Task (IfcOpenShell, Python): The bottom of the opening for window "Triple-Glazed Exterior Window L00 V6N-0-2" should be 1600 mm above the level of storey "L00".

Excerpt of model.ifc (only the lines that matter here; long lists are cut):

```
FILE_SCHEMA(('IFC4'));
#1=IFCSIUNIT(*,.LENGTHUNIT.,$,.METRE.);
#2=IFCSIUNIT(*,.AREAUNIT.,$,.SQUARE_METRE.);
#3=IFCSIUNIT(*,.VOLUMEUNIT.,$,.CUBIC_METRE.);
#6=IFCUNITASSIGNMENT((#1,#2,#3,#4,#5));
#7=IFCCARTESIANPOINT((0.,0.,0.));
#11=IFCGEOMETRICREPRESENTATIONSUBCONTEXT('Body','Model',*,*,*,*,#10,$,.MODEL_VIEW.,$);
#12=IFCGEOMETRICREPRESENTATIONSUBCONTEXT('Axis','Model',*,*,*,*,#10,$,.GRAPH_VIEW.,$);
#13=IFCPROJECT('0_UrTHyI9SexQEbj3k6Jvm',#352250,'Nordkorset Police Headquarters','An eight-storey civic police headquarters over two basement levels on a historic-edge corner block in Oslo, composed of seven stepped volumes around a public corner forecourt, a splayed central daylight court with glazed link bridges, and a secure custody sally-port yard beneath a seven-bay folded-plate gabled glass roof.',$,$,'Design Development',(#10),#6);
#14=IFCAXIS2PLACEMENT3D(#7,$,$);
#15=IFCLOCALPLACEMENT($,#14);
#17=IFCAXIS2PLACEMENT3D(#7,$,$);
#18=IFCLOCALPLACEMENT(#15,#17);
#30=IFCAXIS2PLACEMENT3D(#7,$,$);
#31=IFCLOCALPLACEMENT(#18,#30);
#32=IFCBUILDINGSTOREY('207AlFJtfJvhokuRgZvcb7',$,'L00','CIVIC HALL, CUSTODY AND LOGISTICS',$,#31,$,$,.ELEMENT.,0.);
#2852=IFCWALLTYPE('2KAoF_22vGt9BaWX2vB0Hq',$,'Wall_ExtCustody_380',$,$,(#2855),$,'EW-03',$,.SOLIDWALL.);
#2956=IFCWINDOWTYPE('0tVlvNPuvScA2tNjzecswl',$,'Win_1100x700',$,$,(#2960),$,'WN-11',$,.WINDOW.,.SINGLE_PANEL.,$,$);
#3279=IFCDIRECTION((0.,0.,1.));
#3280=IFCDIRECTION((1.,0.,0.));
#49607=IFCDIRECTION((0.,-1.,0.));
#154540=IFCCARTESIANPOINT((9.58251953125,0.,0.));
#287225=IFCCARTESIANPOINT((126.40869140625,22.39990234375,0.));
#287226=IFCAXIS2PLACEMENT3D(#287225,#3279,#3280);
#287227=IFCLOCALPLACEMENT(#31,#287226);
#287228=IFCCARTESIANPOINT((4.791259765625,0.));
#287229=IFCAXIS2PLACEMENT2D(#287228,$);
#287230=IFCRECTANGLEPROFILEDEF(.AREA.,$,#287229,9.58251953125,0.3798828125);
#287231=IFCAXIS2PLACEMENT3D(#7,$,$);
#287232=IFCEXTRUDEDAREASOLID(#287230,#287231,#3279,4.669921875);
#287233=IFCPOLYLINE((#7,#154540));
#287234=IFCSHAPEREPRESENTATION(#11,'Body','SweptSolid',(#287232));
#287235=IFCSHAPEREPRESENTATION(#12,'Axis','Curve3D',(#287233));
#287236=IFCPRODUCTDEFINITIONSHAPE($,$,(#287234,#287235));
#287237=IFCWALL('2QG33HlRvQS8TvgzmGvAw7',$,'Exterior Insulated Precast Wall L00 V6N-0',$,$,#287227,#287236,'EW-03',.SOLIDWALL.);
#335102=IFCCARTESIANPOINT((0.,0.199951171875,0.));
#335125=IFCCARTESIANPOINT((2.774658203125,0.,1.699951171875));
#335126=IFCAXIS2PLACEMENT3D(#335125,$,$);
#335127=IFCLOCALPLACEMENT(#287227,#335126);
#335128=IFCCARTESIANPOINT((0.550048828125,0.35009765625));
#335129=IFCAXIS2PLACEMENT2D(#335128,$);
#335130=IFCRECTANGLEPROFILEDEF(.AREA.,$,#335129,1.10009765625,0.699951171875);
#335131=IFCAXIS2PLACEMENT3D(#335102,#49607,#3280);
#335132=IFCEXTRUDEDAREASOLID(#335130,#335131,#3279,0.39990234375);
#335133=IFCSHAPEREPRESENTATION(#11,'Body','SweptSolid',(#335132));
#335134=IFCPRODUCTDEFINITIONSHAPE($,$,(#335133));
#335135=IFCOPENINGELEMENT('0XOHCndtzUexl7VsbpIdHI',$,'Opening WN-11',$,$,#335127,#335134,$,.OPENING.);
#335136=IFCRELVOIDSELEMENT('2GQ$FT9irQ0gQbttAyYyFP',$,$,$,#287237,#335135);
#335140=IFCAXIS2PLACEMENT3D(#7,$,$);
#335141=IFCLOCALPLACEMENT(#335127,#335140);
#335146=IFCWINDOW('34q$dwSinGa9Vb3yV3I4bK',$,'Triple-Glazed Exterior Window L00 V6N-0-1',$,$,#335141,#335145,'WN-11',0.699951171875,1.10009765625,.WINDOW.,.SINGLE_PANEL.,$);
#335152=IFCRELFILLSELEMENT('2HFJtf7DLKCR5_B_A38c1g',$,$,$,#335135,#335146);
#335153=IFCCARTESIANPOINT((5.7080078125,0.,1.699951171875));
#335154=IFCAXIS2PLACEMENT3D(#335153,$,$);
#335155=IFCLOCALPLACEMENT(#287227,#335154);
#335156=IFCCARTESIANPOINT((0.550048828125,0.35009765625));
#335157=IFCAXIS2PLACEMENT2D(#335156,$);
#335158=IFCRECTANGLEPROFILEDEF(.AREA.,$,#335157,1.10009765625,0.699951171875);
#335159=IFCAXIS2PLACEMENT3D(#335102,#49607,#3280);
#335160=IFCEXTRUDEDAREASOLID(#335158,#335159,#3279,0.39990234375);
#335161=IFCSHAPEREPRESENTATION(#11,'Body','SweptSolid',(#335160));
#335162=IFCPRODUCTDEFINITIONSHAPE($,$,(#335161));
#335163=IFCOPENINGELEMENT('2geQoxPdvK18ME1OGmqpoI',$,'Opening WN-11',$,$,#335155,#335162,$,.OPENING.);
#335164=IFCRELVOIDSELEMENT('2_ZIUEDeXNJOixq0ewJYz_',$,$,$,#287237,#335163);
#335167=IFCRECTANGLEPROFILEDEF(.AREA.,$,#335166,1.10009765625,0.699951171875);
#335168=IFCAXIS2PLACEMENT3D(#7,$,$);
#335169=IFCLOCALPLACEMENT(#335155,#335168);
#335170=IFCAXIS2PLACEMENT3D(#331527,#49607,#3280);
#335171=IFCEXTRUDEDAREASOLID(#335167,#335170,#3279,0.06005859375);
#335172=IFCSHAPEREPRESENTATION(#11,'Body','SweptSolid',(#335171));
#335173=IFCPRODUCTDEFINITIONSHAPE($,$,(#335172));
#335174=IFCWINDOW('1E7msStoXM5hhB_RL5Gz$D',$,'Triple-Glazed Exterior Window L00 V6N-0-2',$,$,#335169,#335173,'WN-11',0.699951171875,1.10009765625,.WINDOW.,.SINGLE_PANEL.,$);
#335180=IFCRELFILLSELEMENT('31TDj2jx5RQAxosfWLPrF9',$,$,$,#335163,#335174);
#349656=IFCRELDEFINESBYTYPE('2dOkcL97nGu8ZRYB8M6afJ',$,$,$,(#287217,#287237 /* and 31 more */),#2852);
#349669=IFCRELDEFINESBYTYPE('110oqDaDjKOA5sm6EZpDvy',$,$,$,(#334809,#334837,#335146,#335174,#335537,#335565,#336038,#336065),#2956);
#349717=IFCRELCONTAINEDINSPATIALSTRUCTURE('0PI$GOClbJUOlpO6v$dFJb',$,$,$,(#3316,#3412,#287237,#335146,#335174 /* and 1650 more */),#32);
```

```python
import numpy as np
import ifcopenshell
import ifcopenshell.api.geometry
import ifcopenshell.geom
import ifcopenshell.util.element
import ifcopenshell.util.placement
import ifcopenshell.util.shape
import ifcopenshell.util.unit

model = ifcopenshell.open("model.ifc")
unit_scale = ifcopenshell.util.unit.calculate_unit_scale(model)

window = model.by_guid("1E7msStoXM5hhB_RL5Gz$D")
opening = window.FillsVoids[0].RelatingOpeningElement
storey = ifcopenshell.util.element.get_container(window, ifc_class="IfcBuildingStorey")
level = ifcopenshell.util.placement.get_local_placement(storey.ObjectPlacement)[2, 3]

# The opening's origin need not be at the sill, so measure its lowest point.
shape = ifcopenshell.geom.create_shape(ifcopenshell.geom.settings(), opening)
bottom = ifcopenshell.util.shape.get_shape_bottom_elevation(shape, shape.geometry) / unit_scale
dz = level + 1.6 / unit_scale - bottom

shift = np.array([0.0, 0.0, dz])
# The window is placed relative to its opening, so it follows when the opening moves.
matrix = ifcopenshell.util.placement.get_local_placement(opening.ObjectPlacement)
matrix[:3, 3] += shift
ifcopenshell.api.geometry.edit_object_placement(
    model, product=opening, matrix=matrix, is_si=False, should_transform_children=True
)

print(f"moved by {dz * unit_scale:+.3f} m")

model.write("model_rev.ifc")
```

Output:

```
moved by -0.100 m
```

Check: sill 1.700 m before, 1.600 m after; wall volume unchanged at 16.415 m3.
